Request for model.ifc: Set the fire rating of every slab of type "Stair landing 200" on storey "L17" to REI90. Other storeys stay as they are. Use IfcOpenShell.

First a look at what the model holds.

```python
import ifcopenshell
import ifcopenshell.util.element

model = ifcopenshell.open("model.ifc")
print(model.schema)
storey = next(s for s in model.by_type("IfcBuildingStorey") if s.Name == "L17")
slabs = [e for e in ifcopenshell.util.element.get_decomposition(storey) if e.is_a("IfcSlab")]
seen = {}
for e in slabs:
    element_type = ifcopenshell.util.element.get_type(e)
    key = (element_type.Name if element_type != e and element_type else None, ifcopenshell.util.element.get_pset(e, "Pset_SlabCommon", "FireRating"))
    seen[key] = seen.get(key, 0) + 1
for (name, value), count in sorted(seen.items(), key=str):
    print(count, "x", name, "|", value)
```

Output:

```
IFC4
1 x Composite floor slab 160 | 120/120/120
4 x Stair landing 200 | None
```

```python
import ifcopenshell
import ifcopenshell.api.pset
import ifcopenshell.util.element

model = ifcopenshell.open("model.ifc")

storey = next(s for s in model.by_type("IfcBuildingStorey") if s.Name == "L17")
slabs = [e for e in ifcopenshell.util.element.get_decomposition(storey) if e.is_a("IfcSlab")]

count = 0
for e in slabs:
    element_type = ifcopenshell.util.element.get_type(e)
    if element_type in (None, e) or element_type.Name != "Stair landing 200":
        continue
    found = ifcopenshell.util.element.get_pset(e, "Pset_SlabCommon", should_inherit=False)
    if found:
        pset = model.by_id(found["id"])
        if len(ifcopenshell.util.element.get_elements_by_pset(pset)) > 1:
            pset = ifcopenshell.api.pset.unshare_pset(model, products=[e], pset=pset)[0]
    else:
        pset = ifcopenshell.api.pset.add_pset(model, product=e, name="Pset_SlabCommon")
    ifcopenshell.api.pset.edit_pset(model, pset=pset, properties={"FireRating": "REI90"})
    count += 1

print(count, "slabs updated")

model.write("model_edited.ifc")
```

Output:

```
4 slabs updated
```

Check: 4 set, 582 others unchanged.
